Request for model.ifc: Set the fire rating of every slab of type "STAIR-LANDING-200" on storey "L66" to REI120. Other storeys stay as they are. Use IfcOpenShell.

First a look at what the model holds.

```python
import ifcopenshell
import ifcopenshell.util.element

model = ifcopenshell.open("model.ifc")
print(model.schema)
storey = next(s for s in model.by_type("IfcBuildingStorey") if s.Name == "L66")
slabs = [e for e in ifcopenshell.util.element.get_decomposition(storey) if e.is_a("IfcSlab")]
seen = {}
for e in slabs:
    element_type = ifcopenshell.util.element.get_type(e)
    key = (element_type.Name if element_type != e and element_type else None, ifcopenshell.util.element.get_pset(e, "Pset_SlabCommon", "FireRating"))
    seen[key] = seen.get(key, 0) + 1
for (name, value), count in sorted(seen.items(), key=str):
    print(count, "x", name, "|", value)
```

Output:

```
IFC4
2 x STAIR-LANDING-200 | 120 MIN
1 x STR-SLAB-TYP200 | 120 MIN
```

```python
import ifcopenshell
import ifcopenshell.api.pset
import ifcopenshell.util.element

model = ifcopenshell.open("model.ifc")

storey = next(s for s in model.by_type("IfcBuildingStorey") if s.Name == "L66")
slabs = [e for e in ifcopenshell.util.element.get_decomposition(storey) if e.is_a("IfcSlab")]

count = 0
for e in slabs:
    element_type = ifcopenshell.util.element.get_type(e)
    if element_type in (None, e) or element_type.Name != "STAIR-LANDING-200":
        continue
    found = ifcopenshell.util.element.get_pset(e, "Pset_SlabCommon", should_inherit=False)
    if found:
        pset = model.by_id(found["id"])
        if len(ifcopenshell.util.element.get_elements_by_pset(pset)) > 1:
            pset = ifcopenshell.api.pset.unshare_pset(model, products=[e], pset=pset)[0]
    else:
        pset = ifcopenshell.api.pset.add_pset(model, product=e, name="Pset_SlabCommon")
    ifcopenshell.api.pset.edit_pset(model, pset=pset, properties={"FireRating": "REI120"})
    count += 1

print(count, "slabs updated")

model.write("model_v2.ifc")
```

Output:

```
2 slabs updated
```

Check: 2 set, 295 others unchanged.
